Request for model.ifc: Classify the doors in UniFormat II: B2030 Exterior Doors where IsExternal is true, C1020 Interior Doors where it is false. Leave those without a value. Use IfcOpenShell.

First a look at what the model holds.

```python
import ifcopenshell
import ifcopenshell.util.element

model = ifcopenshell.open("model.ifc")
print(model.schema)
print("classifications:", [c.Name for c in model.by_type("IfcClassification")])
values = [ifcopenshell.util.element.get_pset(e, "Pset_DoorCommon", "IsExternal") for e in model.by_type("IfcDoor")]
for value in (True, False, None):
    print("IsExternal", value, values.count(value))
```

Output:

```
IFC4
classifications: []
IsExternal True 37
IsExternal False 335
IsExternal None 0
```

```python
import ifcopenshell
import ifcopenshell.api.classification
import ifcopenshell.util.element

model = ifcopenshell.open("model.ifc")

system = ifcopenshell.api.classification.add_classification(model, classification="UniFormat II")

doors = model.by_type("IfcDoor")
external = {e: ifcopenshell.util.element.get_pset(e, "Pset_DoorCommon", "IsExternal") for e in doors}
for flag, code, name in ((True, "B2030", "Exterior Doors"), (False, "C1020", "Interior Doors")):
    products = [e for e in doors if external[e] is flag]
    ifcopenshell.api.classification.add_reference(
        model, products=products, classification=system, identification=code, name=name
    )
    print(code, len(products))

model.write("model_v2.ifc")
```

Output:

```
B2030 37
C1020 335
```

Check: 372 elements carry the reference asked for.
